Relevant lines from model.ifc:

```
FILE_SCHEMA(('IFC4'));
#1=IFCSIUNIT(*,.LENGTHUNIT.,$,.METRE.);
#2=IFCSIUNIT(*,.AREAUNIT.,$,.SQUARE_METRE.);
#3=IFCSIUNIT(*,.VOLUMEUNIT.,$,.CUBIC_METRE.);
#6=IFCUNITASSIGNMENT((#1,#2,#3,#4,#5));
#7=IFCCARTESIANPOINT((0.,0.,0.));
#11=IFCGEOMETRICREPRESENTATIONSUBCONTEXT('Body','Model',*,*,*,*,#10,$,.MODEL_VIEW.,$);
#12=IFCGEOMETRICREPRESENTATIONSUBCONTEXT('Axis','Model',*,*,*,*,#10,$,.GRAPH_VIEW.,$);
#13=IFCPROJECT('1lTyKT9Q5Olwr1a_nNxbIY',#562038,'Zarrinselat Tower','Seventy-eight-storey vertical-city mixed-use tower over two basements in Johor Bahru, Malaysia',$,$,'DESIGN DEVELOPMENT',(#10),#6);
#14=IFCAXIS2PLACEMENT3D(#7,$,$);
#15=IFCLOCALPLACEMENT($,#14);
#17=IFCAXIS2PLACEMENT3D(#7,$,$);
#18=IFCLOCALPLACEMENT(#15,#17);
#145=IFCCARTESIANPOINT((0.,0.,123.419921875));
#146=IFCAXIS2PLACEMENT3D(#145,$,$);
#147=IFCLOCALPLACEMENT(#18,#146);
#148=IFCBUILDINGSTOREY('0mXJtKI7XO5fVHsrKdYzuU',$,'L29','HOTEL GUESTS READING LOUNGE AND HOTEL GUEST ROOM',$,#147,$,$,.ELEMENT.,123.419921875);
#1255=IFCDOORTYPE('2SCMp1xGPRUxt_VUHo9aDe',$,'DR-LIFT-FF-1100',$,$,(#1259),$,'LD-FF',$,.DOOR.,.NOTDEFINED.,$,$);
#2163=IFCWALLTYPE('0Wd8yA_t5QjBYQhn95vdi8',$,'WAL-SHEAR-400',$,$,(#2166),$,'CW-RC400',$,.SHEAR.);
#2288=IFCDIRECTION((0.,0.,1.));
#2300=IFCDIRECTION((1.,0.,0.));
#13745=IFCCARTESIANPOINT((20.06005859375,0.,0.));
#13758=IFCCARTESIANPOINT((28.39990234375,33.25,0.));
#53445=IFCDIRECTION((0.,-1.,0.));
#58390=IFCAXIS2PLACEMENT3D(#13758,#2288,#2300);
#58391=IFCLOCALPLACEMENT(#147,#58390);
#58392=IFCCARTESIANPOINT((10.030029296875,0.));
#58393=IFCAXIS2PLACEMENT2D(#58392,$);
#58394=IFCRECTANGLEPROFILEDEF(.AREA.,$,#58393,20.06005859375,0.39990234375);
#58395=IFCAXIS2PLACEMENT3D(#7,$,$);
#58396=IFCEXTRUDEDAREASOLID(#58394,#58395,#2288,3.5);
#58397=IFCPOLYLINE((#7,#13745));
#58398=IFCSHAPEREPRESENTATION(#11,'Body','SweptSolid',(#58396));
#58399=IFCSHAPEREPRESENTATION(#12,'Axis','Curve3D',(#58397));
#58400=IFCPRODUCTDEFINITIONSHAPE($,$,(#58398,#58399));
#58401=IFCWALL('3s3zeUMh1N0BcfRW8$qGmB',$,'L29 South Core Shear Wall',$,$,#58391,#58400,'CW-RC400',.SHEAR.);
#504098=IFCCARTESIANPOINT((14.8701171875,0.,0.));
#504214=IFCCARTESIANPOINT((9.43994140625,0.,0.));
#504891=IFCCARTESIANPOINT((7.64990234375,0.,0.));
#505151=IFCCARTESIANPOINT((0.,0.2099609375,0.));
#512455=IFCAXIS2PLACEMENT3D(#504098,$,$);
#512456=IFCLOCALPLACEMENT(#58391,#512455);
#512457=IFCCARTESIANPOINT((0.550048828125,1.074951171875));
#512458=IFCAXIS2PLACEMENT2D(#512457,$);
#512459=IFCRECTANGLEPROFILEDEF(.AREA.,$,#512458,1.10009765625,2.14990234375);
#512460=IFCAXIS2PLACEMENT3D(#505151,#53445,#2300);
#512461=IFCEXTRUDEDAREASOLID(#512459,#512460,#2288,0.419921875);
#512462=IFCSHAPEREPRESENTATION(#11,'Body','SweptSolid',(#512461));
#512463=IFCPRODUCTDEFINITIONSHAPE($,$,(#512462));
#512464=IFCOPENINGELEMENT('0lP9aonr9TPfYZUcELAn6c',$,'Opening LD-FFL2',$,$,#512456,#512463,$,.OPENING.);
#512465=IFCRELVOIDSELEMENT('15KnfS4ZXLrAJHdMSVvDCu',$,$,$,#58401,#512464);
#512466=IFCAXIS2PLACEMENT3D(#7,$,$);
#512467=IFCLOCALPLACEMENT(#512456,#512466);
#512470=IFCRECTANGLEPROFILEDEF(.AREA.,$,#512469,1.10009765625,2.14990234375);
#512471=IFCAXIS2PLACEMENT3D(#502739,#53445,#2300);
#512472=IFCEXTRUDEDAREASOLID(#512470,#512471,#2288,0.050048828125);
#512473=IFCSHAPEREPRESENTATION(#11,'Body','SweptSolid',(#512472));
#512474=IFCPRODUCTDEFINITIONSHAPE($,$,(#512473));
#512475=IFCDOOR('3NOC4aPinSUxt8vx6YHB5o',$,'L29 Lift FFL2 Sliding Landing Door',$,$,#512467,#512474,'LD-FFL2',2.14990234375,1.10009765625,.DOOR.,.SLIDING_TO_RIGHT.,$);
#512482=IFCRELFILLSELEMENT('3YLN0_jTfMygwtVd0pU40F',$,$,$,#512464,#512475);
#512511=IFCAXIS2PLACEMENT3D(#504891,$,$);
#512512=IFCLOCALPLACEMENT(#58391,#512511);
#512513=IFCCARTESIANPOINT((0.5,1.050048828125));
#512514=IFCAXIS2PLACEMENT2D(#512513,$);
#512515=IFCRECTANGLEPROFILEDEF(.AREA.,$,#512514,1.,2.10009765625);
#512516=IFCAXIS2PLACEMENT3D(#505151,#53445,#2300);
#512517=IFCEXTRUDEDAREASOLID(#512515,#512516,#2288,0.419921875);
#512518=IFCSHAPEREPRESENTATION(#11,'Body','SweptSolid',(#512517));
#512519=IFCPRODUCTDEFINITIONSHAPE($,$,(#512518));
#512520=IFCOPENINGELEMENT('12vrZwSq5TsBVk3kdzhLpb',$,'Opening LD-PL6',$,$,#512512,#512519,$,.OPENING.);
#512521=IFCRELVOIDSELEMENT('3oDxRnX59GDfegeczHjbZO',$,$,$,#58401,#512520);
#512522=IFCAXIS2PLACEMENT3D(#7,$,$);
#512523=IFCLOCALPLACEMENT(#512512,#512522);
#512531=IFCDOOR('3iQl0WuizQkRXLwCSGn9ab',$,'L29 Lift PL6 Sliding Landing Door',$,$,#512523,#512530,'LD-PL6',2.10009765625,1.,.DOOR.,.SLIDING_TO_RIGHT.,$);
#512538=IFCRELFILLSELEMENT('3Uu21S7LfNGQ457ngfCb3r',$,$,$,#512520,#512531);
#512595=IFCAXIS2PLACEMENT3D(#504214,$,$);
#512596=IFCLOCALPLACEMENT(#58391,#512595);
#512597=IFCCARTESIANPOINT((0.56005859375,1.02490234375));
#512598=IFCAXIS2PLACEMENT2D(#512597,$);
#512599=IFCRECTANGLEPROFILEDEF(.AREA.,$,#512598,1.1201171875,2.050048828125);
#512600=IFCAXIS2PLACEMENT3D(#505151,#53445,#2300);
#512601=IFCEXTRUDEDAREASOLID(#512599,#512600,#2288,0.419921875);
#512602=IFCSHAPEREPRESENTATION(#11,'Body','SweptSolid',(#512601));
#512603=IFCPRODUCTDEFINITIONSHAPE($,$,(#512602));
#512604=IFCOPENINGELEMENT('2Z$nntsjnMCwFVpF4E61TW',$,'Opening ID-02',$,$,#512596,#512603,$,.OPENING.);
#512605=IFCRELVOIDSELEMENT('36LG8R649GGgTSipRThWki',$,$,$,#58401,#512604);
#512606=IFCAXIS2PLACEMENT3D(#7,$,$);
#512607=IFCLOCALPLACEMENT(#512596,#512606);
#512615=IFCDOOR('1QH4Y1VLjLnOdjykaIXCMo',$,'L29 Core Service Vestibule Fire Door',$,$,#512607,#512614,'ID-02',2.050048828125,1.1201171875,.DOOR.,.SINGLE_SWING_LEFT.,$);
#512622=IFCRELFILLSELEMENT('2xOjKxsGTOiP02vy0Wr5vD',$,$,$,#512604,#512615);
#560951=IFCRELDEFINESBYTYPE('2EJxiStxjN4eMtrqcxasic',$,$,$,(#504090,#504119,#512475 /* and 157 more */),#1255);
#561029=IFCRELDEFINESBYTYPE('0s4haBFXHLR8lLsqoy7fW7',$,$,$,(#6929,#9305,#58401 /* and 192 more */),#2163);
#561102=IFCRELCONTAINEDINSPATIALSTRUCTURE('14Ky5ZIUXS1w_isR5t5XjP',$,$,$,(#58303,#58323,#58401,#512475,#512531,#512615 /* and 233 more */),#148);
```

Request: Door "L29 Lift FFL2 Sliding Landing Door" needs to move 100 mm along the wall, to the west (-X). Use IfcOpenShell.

```python
import ifcopenshell
import ifcopenshell.api.geometry
import ifcopenshell.util.placement
import ifcopenshell.util.unit

model = ifcopenshell.open("model.ifc")
unit_scale = ifcopenshell.util.unit.calculate_unit_scale(model)

door = model.by_guid("3NOC4aPinSUxt8vx6YHB5o")
opening = door.FillsVoids[0].RelatingOpeningElement
wall = opening.VoidsElements[0].RelatingBuildingElement

wall_matrix = ifcopenshell.util.placement.get_local_placement(wall.ObjectPlacement)
shift = wall_matrix[:3, 0] * -0.1 / unit_scale
before = ifcopenshell.util.placement.get_local_placement(door.ObjectPlacement)[:3, 3].copy()

# The door is placed relative to its opening, so it follows when the opening moves.
matrix = ifcopenshell.util.placement.get_local_placement(opening.ObjectPlacement)
matrix[:3, 3] += shift
ifcopenshell.api.geometry.edit_object_placement(
    model, product=opening, matrix=matrix, is_si=False, should_transform_children=True
)

after = ifcopenshell.util.placement.get_local_placement(door.ObjectPlacement)[:3, 3]
print("door moved by", (after - before).round(3) + 0.0)

model.write("model_rev.ifc")
```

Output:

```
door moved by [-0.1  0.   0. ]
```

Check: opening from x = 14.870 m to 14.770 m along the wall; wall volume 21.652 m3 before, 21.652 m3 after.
